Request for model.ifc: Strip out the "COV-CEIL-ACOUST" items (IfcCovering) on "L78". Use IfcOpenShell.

First a look at what the model holds.

```python
import ifcopenshell
import ifcopenshell.util.element

model = ifcopenshell.open("model.ifc")
print(model.schema)
storey = next(s for s in model.by_type("IfcBuildingStorey") if s.Name == "L78")
coverings = [e for e in ifcopenshell.util.element.get_decomposition(storey) if e.is_a("IfcCovering")]
seen = {}
for e in coverings:
    element_type = ifcopenshell.util.element.get_type(e)
    name = element_type.Name if element_type not in (None, e) else None
    seen[name] = seen.get(name, 0) + 1
for name, count in sorted(seen.items(), key=str):
    print(count, "x", name)
```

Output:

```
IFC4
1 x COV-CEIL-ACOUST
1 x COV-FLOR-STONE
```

```python
import ifcopenshell
import ifcopenshell.api.root
import ifcopenshell.util.element

model = ifcopenshell.open("model.ifc")

storey = next(s for s in model.by_type("IfcBuildingStorey") if s.Name == "L78")
coverings = [e for e in ifcopenshell.util.element.get_decomposition(storey) if e.is_a("IfcCovering")]
targets = [e for e in coverings if (t := ifcopenshell.util.element.get_type(e)) not in (None, e) and t.Name == "COV-CEIL-ACOUST"]

for e in targets:
    ifcopenshell.api.root.remove_product(model, product=e)
print(len(targets), "removed")

model.write("model-out.ifc")
```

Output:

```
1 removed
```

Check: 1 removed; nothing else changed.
